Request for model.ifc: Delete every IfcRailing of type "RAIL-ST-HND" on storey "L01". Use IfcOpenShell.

First a look at what the model holds.

```python
import ifcopenshell
import ifcopenshell.util.element

model = ifcopenshell.open("model.ifc")
print(model.schema)
storey = next(s for s in model.by_type("IfcBuildingStorey") if s.Name == "L01")
railings = [e for e in ifcopenshell.util.element.get_decomposition(storey) if e.is_a("IfcRailing")]
seen = {}
for e in railings:
    element_type = ifcopenshell.util.element.get_type(e)
    name = element_type.Name if element_type not in (None, e) else None
    seen[name] = seen.get(name, 0) + 1
for name, count in sorted(seen.items(), key=str):
    print(count, "x", name)
```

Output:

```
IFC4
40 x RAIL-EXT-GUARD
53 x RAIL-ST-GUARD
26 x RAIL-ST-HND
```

```python
import ifcopenshell
import ifcopenshell.api.root
import ifcopenshell.util.element

model = ifcopenshell.open("model.ifc")

storey = next(s for s in model.by_type("IfcBuildingStorey") if s.Name == "L01")
railings = [e for e in ifcopenshell.util.element.get_decomposition(storey) if e.is_a("IfcRailing")]
targets = [e for e in railings if (t := ifcopenshell.util.element.get_type(e)) not in (None, e) and t.Name == "RAIL-ST-HND"]

for e in targets:
    ifcopenshell.api.root.remove_product(model, product=e)
print(len(targets), "removed")

model.write("model_updated.ifc")
```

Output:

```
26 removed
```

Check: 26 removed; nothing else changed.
